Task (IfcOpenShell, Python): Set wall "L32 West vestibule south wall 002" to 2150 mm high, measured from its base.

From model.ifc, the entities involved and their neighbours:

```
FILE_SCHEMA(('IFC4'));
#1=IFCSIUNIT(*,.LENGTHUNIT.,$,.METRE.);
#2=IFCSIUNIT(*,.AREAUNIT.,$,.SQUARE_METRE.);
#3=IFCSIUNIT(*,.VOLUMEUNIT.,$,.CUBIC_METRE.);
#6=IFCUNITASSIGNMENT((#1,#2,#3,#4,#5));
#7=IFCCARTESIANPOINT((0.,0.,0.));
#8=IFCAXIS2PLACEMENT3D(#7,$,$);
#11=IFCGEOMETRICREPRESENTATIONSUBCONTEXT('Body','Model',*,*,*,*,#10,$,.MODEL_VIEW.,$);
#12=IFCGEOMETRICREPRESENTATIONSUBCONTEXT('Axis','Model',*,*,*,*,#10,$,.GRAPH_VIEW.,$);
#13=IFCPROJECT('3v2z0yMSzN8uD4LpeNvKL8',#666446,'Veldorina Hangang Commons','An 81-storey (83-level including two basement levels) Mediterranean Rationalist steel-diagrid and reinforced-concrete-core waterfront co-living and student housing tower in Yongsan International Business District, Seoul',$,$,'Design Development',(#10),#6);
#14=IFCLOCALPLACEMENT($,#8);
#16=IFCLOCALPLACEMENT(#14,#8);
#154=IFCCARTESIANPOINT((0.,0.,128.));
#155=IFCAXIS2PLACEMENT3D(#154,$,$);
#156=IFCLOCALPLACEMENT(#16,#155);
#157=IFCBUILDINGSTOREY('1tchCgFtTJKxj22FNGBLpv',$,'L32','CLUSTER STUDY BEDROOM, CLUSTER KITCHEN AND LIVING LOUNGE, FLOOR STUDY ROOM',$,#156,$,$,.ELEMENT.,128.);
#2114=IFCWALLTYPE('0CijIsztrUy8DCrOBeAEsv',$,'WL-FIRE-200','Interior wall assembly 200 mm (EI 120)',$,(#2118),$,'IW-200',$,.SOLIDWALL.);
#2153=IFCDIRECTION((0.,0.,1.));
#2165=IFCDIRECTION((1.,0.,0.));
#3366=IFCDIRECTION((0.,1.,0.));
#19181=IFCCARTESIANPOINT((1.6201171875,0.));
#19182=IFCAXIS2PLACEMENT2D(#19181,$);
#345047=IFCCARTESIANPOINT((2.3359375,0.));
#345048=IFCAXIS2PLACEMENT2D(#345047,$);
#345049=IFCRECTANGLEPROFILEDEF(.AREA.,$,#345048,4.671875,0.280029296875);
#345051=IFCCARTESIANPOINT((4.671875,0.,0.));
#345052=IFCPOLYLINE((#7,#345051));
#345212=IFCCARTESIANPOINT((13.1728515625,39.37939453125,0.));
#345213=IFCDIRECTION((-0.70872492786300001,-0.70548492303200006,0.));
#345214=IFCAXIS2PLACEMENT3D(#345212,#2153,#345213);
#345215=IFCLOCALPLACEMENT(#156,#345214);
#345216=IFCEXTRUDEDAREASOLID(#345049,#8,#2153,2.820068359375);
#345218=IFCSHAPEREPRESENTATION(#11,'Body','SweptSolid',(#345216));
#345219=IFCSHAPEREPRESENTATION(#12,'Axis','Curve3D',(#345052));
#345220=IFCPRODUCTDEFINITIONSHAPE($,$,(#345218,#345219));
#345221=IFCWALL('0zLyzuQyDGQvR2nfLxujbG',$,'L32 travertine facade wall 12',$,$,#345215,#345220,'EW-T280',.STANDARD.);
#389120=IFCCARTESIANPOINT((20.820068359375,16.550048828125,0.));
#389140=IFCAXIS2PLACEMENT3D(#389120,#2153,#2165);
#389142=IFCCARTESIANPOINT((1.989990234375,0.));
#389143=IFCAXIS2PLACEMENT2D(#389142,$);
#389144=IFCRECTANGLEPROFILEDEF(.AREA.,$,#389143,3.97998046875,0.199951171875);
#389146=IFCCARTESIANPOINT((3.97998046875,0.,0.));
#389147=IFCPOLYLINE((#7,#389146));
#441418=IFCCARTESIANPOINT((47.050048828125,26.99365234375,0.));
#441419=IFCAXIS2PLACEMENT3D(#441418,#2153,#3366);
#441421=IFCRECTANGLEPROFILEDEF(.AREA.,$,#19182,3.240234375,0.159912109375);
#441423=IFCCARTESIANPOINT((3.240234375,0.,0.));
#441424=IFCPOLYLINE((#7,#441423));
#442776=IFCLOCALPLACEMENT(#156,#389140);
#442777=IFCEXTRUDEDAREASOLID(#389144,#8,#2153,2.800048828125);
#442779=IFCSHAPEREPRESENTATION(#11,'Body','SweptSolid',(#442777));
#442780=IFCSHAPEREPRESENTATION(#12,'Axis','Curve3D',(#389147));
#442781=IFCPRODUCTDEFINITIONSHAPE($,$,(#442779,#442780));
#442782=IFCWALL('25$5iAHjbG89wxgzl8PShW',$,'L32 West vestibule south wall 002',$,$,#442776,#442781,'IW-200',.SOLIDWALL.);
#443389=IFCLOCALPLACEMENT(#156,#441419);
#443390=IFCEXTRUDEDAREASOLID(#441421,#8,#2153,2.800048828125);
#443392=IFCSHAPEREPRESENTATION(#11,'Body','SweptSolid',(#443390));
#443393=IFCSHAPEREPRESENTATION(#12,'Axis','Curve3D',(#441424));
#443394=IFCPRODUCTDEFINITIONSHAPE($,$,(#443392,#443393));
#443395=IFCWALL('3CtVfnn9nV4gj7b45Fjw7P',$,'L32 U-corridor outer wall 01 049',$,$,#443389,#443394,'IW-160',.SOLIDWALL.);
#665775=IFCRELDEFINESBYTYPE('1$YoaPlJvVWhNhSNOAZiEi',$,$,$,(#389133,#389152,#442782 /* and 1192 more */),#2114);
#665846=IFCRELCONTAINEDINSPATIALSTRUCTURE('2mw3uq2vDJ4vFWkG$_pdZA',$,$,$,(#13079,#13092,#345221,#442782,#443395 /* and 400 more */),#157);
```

```python
import ifcopenshell
import ifcopenshell.geom
import ifcopenshell.util.representation
import ifcopenshell.util.shape
import ifcopenshell.util.unit

model = ifcopenshell.open("model.ifc")
unit_scale = ifcopenshell.util.unit.calculate_unit_scale(model)
settings = ifcopenshell.geom.settings()


def volume(element):
    """Net volume in cubic metres, openings subtracted."""
    shape = ifcopenshell.geom.create_shape(settings, element)
    return ifcopenshell.util.shape.get_volume(shape.geometry)


wall = model.by_guid("25$5iAHjbG89wxgzl8PShW")
before = volume(wall)

body = ifcopenshell.util.representation.get_representation(wall, "Model", "Body")
solid = body.Items[0]
old_height = solid.Depth
solid.Depth = 2.15 / unit_scale
after = volume(wall)

print(f"height {old_height:g} -> {solid.Depth:g}, volume {before:.3f} -> {after:.3f} m3")

model.write("model_v2.ifc")
```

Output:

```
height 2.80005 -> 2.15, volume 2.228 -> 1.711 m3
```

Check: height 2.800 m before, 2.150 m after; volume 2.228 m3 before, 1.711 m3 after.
